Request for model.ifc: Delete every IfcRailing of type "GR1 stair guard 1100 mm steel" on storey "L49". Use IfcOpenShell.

First a look at what the model holds.

```python
import ifcopenshell
import ifcopenshell.util.element

model = ifcopenshell.open("model.ifc")
print(model.schema)
storey = next(s for s in model.by_type("IfcBuildingStorey") if s.Name == "L49")
railings = [e for e in ifcopenshell.util.element.get_decomposition(storey) if e.is_a("IfcRailing")]
seen = {}
for e in railings:
    element_type = ifcopenshell.util.element.get_type(e)
    name = element_type.Name if element_type not in (None, e) else None
    seen[name] = seen.get(name, 0) + 1
for name, count in sorted(seen.items(), key=str):
    print(count, "x", name)
```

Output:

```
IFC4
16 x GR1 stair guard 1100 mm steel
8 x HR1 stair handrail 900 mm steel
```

```python
import ifcopenshell
import ifcopenshell.api.root
import ifcopenshell.util.element

model = ifcopenshell.open("model.ifc")

storey = next(s for s in model.by_type("IfcBuildingStorey") if s.Name == "L49")
railings = [e for e in ifcopenshell.util.element.get_decomposition(storey) if e.is_a("IfcRailing")]
targets = [e for e in railings if (t := ifcopenshell.util.element.get_type(e)) not in (None, e) and t.Name == "GR1 stair guard 1100 mm steel"]

for e in targets:
    ifcopenshell.api.root.remove_product(model, product=e)
print(len(targets), "removed")

model.write("model_edited.ifc")
```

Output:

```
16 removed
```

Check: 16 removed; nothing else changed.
